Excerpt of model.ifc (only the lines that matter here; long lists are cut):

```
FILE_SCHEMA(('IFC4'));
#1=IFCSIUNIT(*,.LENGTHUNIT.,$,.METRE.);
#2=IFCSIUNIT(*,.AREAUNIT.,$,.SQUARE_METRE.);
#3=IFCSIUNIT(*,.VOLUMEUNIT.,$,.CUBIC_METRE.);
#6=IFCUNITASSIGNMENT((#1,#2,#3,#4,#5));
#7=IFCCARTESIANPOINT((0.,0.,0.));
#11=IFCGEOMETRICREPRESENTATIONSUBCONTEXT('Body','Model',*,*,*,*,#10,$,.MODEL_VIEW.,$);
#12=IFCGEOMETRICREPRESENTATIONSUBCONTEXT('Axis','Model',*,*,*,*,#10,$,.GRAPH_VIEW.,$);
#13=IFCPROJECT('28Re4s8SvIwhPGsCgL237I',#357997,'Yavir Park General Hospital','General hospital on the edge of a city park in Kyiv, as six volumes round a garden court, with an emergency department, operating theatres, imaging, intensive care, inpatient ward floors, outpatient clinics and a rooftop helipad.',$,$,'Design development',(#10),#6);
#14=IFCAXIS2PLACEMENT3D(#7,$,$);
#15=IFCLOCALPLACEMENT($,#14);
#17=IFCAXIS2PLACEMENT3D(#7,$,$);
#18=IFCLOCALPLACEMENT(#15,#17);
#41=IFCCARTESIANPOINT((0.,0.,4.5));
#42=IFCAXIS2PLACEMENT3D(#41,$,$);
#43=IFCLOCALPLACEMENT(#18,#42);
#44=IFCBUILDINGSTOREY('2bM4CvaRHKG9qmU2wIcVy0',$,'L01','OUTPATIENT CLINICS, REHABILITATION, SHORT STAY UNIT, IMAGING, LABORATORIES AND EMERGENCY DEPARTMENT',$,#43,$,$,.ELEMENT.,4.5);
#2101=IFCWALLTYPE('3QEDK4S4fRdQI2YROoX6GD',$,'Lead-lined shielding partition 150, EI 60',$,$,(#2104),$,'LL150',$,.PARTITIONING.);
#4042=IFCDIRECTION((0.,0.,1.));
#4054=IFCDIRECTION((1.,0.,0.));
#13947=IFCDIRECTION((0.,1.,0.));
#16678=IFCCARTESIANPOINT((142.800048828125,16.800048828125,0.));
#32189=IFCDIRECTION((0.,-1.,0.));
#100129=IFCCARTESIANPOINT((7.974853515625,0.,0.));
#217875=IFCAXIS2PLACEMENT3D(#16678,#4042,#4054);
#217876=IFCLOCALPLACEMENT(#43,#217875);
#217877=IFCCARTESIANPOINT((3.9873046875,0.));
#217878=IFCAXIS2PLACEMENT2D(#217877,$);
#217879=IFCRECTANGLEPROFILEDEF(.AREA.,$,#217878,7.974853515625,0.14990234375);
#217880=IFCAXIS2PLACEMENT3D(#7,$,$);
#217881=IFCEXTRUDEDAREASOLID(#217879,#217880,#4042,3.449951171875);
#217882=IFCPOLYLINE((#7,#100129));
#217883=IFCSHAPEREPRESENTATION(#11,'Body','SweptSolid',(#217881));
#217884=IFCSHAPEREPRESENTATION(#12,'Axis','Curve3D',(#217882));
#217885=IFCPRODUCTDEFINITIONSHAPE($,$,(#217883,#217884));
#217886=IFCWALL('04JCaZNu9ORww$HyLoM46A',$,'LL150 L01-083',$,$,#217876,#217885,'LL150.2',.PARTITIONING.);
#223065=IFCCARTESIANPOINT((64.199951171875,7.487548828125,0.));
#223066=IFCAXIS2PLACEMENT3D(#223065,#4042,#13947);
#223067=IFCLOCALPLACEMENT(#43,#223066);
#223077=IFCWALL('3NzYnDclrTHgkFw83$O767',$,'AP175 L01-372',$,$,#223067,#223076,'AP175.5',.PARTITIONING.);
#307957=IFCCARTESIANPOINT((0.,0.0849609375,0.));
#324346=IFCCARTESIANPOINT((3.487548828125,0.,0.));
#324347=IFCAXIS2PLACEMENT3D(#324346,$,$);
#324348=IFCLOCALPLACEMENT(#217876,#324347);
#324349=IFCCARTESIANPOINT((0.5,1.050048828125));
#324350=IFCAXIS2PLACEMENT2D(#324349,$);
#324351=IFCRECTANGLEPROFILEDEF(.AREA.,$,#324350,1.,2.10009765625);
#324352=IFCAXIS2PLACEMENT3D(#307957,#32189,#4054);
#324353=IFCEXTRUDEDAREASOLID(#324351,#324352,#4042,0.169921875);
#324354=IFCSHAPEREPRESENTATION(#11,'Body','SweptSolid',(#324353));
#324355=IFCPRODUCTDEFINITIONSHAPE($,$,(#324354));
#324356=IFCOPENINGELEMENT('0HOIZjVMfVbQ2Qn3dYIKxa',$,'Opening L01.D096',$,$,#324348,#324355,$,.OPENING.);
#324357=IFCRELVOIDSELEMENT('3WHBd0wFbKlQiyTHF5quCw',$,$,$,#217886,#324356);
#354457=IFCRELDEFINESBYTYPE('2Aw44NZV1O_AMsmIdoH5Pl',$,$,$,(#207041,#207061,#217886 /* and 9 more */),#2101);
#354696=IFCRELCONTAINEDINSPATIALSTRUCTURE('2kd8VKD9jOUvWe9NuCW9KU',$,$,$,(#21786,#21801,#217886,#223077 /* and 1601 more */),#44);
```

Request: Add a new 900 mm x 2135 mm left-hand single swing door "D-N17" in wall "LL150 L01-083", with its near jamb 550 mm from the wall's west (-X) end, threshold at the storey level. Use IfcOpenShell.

```python
import numpy as np
import ifcopenshell
import ifcopenshell.api.feature
import ifcopenshell.api.geometry
import ifcopenshell.api.root
import ifcopenshell.api.spatial
import ifcopenshell.geom
import ifcopenshell.util.element
import ifcopenshell.util.placement
import ifcopenshell.util.representation
import ifcopenshell.util.shape
import ifcopenshell.util.unit

model = ifcopenshell.open("model.ifc")
unit_scale = ifcopenshell.util.unit.calculate_unit_scale(model)
settings = ifcopenshell.geom.settings()


def volume(element):
    """Net volume in cubic metres, openings subtracted."""
    shape = ifcopenshell.geom.create_shape(settings, element)
    return ifcopenshell.util.shape.get_volume(shape.geometry)


wall = model.by_guid("04JCaZNu9ORww$HyLoM46A")
storey = ifcopenshell.util.element.get_container(wall, ifc_class="IfcBuildingStorey")
context = ifcopenshell.util.representation.get_context(model, "Model", "Body", "MODEL_VIEW")
before = volume(wall)

width, height, from_end, sill = 0.9, 2.135, 0.55, 0.0  # metres

# The wall runs along its own X axis, and the end named is its -X end.
wall_shape = ifcopenshell.geom.create_shape(settings, wall)
x, y, z = ifcopenshell.util.shape.get_vertices(wall_shape.geometry).T
start = x.min() + from_end
face, thickness = float(y.min()), float(y.max() - y.min())
wall_matrix = ifcopenshell.util.placement.get_local_placement(wall.ObjectPlacement)
level = ifcopenshell.util.placement.get_local_placement(storey.ObjectPlacement)[2, 3]


def in_wall(x, y):
    """Placement at x, y metres in the wall's axes, at sill height."""
    matrix = wall_matrix.copy()
    matrix[:, 3] = wall_matrix @ np.array([x / unit_scale, y / unit_scale, 0.0, 1.0])
    matrix[2, 3] = level + sill / unit_scale
    return matrix


# Opening: a box that overshoots both wall faces by 50 mm.
opening = ifcopenshell.api.root.create_entity(model, ifc_class="IfcOpeningElement", predefined_type="OPENING")
box = ifcopenshell.api.geometry.add_wall_representation(
    model, context=context, length=width, height=height, thickness=thickness + 0.1
)
ifcopenshell.api.geometry.assign_representation(model, product=opening, representation=box)
ifcopenshell.api.geometry.edit_object_placement(model, product=opening, matrix=in_wall(start, face - 0.05), is_si=False)
ifcopenshell.api.feature.add_feature(model, feature=opening, element=wall)

door = ifcopenshell.api.root.create_entity(model, ifc_class="IfcDoor", name="D-N17", predefined_type="DOOR")
door.OverallWidth, door.OverallHeight = width / unit_scale, height / unit_scale
door.OperationType = "SINGLE_SWING_LEFT"
body = ifcopenshell.api.geometry.add_door_representation(
    model,
    context=context,
    overall_width=door.OverallWidth,
    overall_height=door.OverallHeight,
    operation_type="SINGLE_SWING_LEFT",
    lining_properties={"LiningDepth": thickness / unit_scale, "ThresholdDepth": thickness / unit_scale},
)
ifcopenshell.api.geometry.assign_representation(model, product=door, representation=body)
ifcopenshell.api.spatial.assign_container(model, products=[door], relating_structure=storey)
ifcopenshell.api.feature.add_filling(model, opening=opening, element=door)

# The lining spans the wall, so the door starts at the wall face.
ifcopenshell.api.geometry.edit_object_placement(model, product=door, matrix=in_wall(start, face), is_si=False)

after = volume(wall)

print(f"wall volume {before:.3f} -> {after:.3f} m3")

model.write("model_edited.ifc")
```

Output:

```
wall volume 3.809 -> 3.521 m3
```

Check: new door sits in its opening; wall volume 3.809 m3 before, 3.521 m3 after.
